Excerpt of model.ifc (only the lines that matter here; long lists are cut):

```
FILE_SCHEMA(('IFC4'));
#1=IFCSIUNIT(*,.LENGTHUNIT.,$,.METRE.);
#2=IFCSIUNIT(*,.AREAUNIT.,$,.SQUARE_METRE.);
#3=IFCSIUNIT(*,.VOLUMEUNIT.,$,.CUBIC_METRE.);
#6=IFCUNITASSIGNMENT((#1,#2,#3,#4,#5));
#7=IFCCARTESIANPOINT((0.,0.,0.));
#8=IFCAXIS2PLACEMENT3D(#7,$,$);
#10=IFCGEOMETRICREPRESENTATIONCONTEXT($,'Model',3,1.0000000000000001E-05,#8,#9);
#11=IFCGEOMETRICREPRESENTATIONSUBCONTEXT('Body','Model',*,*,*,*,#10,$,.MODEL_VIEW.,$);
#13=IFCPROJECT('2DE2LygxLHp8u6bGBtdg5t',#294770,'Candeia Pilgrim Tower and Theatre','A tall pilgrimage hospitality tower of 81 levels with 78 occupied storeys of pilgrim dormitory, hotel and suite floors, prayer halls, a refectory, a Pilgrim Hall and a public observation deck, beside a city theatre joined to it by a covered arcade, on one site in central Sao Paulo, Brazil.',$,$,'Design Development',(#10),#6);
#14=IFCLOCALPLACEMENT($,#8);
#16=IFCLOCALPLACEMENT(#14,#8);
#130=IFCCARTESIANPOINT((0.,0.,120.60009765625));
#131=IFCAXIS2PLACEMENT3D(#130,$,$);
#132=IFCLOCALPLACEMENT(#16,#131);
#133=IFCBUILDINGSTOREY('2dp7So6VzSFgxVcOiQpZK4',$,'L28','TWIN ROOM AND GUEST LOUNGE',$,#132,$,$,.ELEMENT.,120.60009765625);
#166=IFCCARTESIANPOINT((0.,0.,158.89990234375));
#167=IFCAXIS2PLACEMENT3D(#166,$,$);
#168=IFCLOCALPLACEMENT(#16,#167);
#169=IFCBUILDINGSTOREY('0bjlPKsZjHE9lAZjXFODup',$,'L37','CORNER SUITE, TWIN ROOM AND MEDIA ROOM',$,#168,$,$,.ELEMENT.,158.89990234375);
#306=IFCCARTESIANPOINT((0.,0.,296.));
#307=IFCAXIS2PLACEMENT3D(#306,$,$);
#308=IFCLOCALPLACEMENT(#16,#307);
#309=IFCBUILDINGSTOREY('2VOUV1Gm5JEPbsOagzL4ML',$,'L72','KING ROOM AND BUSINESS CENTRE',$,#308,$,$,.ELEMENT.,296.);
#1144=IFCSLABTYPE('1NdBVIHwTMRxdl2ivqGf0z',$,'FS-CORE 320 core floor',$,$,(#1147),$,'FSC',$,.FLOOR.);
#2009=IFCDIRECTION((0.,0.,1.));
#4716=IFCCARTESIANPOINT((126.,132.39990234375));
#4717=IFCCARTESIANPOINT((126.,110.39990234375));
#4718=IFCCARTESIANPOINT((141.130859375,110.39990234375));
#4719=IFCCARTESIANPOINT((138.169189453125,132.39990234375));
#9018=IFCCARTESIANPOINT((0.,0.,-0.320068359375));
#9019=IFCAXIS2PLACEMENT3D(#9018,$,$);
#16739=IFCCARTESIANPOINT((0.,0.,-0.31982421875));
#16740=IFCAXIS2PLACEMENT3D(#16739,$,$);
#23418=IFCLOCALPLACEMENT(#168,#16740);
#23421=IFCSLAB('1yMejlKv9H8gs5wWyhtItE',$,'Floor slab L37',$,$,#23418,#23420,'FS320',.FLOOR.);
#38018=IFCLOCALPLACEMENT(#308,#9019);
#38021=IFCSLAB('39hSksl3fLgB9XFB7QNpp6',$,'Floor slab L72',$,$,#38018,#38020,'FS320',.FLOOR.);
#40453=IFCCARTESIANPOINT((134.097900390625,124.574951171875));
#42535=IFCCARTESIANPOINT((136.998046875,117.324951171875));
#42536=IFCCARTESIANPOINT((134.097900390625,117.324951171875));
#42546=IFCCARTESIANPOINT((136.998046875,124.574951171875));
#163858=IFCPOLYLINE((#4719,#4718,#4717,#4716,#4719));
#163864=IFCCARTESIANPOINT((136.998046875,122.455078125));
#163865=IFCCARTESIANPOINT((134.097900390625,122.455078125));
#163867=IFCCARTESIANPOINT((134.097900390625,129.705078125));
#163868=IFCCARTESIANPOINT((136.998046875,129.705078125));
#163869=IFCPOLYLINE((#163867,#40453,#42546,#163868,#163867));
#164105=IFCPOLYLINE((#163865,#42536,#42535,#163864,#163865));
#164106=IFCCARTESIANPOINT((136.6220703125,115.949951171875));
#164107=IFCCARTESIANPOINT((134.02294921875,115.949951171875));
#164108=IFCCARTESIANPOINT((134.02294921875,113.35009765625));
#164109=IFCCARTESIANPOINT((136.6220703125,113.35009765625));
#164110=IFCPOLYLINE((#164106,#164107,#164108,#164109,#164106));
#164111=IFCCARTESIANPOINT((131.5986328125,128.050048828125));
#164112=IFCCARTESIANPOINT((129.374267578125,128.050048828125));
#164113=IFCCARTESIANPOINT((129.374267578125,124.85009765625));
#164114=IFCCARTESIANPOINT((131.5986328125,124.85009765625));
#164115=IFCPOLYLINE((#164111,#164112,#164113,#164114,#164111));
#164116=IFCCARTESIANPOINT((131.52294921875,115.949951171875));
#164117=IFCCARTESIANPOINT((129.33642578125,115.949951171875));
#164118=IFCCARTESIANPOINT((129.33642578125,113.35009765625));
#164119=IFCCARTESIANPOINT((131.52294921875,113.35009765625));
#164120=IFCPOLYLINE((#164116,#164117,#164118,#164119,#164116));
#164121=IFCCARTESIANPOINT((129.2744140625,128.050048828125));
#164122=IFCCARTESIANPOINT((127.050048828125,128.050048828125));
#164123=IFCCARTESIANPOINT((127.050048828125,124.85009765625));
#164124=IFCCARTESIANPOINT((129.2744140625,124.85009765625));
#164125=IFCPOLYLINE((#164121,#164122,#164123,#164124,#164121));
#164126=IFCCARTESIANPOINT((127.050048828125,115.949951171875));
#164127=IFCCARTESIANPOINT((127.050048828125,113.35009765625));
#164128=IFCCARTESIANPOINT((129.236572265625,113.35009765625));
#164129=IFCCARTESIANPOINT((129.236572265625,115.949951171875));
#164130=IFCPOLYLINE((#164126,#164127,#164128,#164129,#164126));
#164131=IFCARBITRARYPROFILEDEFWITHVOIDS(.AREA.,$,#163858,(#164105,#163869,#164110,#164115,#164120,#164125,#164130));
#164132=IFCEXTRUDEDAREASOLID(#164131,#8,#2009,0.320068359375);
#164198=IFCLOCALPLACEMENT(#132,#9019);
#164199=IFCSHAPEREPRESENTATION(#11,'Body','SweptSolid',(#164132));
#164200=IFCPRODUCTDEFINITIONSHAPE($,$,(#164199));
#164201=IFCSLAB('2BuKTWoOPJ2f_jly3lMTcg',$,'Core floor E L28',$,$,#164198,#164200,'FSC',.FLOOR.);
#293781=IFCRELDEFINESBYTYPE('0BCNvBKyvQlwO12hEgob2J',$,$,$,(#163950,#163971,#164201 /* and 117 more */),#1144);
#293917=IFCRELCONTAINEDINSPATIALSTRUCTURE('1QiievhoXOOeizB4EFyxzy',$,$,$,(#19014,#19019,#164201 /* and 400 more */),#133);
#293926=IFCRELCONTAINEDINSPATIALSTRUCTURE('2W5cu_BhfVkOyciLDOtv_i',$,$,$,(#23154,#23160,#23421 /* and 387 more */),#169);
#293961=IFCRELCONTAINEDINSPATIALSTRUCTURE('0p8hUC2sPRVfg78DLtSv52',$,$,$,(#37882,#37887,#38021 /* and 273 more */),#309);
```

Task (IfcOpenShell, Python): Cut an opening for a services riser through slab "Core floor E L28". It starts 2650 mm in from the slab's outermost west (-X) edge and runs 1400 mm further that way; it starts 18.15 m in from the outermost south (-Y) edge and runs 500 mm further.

```python
import numpy as np
import ifcopenshell
import ifcopenshell.api.feature
import ifcopenshell.api.geometry
import ifcopenshell.api.root
import ifcopenshell.geom
import ifcopenshell.util.placement
import ifcopenshell.util.representation
import ifcopenshell.util.shape
import ifcopenshell.util.unit

model = ifcopenshell.open("model.ifc")
unit_scale = ifcopenshell.util.unit.calculate_unit_scale(model)
settings = ifcopenshell.geom.settings()


def volume(element):
    """Net volume in cubic metres, openings subtracted."""
    shape = ifcopenshell.geom.create_shape(settings, element)
    return ifcopenshell.util.shape.get_volume(shape.geometry)


slab = model.by_id(164201)
before = volume(slab)

# Extent in the slab's own axes, in metres. The edges named are its -X and -Y sides.
slab_shape = ifcopenshell.geom.create_shape(settings, slab)
vertices = ifcopenshell.util.shape.get_vertices(slab_shape.geometry)
x_min, y_min, bottom = vertices.min(axis=0)
top = vertices[:, 2].max()

opening = ifcopenshell.api.root.create_entity(model, ifc_class="IfcOpeningElement", name="Services riser opening", predefined_type="OPENING")
context = ifcopenshell.util.representation.get_context(model, "Model", "Body", "MODEL_VIEW")
width, depth = 1.4, 0.5
outline = [(0.0, 0.0), (width, 0.0), (width, depth), (0.0, depth), (0.0, 0.0)]
# Overshoot both faces by 50 mm so the cut is clean.
shape = ifcopenshell.api.geometry.add_slab_representation(
    model, context=context, depth=top - bottom + 0.1, polyline=outline
)
ifcopenshell.api.geometry.assign_representation(model, product=opening, representation=shape)

matrix = ifcopenshell.util.placement.get_local_placement(slab.ObjectPlacement)
matrix[:, 3] = matrix @ np.append(np.array([x_min + 2.65, y_min + 18.15, bottom - 0.05]) / unit_scale, 1.0)
ifcopenshell.api.geometry.edit_object_placement(model, product=opening, matrix=matrix, is_si=False)
ifcopenshell.api.feature.add_feature(model, feature=opening, element=slab)

after = volume(slab)

print(f"slab volume {before:.3f} -> {after:.3f} m3")

model.write("model_rev.ifc")
```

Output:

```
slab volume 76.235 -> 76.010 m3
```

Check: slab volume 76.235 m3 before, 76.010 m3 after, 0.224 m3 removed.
